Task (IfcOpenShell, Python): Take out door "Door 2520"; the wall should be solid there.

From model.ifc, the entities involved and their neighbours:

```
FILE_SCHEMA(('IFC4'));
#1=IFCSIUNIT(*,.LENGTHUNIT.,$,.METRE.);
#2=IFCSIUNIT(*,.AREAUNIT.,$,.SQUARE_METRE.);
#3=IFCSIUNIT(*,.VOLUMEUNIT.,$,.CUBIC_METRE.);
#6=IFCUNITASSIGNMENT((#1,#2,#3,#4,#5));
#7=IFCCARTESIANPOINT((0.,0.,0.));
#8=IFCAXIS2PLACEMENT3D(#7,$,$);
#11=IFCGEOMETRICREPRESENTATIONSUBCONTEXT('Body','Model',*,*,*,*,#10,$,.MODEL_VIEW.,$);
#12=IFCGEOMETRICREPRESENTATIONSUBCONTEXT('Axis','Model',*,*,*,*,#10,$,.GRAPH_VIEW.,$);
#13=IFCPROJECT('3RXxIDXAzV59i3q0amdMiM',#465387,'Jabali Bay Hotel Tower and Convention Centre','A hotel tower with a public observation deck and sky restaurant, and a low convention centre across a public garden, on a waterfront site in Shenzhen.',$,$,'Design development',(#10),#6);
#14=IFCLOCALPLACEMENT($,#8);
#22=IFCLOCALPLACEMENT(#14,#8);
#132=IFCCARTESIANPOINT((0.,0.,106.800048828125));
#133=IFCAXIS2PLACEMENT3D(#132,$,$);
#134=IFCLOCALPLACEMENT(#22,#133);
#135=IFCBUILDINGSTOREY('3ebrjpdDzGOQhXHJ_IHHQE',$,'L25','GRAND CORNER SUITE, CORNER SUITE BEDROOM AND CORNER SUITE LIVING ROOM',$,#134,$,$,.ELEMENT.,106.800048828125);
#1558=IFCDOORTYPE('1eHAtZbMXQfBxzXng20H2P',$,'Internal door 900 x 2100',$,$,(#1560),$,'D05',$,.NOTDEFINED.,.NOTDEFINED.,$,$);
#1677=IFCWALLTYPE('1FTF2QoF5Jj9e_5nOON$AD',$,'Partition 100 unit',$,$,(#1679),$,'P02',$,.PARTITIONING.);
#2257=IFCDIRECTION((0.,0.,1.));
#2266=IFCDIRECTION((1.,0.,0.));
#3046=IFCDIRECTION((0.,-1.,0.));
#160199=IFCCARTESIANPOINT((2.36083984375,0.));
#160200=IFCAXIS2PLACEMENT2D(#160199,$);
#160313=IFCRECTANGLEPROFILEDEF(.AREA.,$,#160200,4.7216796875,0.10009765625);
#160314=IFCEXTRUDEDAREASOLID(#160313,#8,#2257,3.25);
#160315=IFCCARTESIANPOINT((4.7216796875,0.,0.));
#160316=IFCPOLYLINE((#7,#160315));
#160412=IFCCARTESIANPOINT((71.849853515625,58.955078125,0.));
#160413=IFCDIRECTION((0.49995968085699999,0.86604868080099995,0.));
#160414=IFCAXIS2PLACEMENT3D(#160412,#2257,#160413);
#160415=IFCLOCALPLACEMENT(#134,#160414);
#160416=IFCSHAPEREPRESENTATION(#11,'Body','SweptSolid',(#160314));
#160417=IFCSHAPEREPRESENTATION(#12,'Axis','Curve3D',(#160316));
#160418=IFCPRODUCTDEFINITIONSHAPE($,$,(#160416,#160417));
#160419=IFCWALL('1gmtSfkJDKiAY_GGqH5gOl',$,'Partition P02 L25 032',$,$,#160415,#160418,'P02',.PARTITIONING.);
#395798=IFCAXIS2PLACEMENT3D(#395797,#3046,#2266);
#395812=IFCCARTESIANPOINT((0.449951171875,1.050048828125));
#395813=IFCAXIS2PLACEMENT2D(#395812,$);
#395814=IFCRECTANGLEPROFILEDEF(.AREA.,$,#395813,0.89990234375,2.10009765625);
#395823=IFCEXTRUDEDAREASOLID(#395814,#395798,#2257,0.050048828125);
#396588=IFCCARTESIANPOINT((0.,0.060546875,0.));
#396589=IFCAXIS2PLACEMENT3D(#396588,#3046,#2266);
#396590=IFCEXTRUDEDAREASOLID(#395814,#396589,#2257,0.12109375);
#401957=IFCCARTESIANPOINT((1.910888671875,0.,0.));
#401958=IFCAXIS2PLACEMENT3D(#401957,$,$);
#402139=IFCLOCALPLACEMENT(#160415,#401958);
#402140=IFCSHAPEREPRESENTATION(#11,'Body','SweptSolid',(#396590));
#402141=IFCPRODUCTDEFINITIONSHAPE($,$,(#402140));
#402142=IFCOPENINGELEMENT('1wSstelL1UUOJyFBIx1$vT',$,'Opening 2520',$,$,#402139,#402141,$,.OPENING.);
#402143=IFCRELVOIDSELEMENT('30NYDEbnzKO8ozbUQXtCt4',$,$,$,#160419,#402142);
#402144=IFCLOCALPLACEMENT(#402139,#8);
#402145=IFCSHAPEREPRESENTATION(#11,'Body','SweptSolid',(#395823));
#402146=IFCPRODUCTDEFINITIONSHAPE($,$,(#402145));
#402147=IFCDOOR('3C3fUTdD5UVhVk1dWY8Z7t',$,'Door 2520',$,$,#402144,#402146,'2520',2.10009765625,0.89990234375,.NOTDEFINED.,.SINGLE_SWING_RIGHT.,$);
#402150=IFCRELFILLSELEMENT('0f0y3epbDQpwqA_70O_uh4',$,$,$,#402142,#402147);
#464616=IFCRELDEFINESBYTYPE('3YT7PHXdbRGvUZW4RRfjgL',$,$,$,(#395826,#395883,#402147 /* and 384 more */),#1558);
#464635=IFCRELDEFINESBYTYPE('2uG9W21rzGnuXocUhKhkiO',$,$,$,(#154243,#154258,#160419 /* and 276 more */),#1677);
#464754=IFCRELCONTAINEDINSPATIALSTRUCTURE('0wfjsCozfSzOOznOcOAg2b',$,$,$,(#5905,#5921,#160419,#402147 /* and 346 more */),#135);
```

```python
import ifcopenshell
import ifcopenshell.api.feature
import ifcopenshell.api.root
import ifcopenshell.geom
import ifcopenshell.util.shape

model = ifcopenshell.open("model.ifc")
settings = ifcopenshell.geom.settings()


def volume(element):
    """Net volume in cubic metres, openings subtracted."""
    shape = ifcopenshell.geom.create_shape(settings, element)
    return ifcopenshell.util.shape.get_volume(shape.geometry)


door = model.by_id(402147)
opening = door.FillsVoids[0].RelatingOpeningElement
wall = opening.VoidsElements[0].RelatingBuildingElement
before = volume(wall)

ifcopenshell.api.root.remove_product(model, product=door)
ifcopenshell.api.feature.remove_feature(model, feature=opening)

after = volume(wall)

print(f"wall volume {before:.3f} -> {after:.3f} m3")

model.write("model_edited.ifc")
```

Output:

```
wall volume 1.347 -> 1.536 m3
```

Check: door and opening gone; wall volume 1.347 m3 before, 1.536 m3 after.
